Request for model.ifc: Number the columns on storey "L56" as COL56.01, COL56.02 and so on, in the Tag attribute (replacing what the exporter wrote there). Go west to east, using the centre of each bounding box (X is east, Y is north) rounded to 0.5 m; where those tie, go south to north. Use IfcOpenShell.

First a look at what the model holds.

```python
import ifcopenshell
import ifcopenshell.util.element
import ifcopenshell.util.placement

model = ifcopenshell.open("model.ifc")
print(model.schema)
storey = next(s for s in model.by_type("IfcBuildingStorey") if s.Name == "L56")
columns = [e for e in ifcopenshell.util.element.get_decomposition(storey) if e.is_a("IfcColumn")]
for e in sorted(columns, key=lambda e: e.id()):
    origin = ifcopenshell.util.placement.get_local_placement(e.ObjectPlacement)[:3, 3]
    print(e.id(), e.Tag, e.Name, origin.round(2) + 0.0, sep=" | ")
```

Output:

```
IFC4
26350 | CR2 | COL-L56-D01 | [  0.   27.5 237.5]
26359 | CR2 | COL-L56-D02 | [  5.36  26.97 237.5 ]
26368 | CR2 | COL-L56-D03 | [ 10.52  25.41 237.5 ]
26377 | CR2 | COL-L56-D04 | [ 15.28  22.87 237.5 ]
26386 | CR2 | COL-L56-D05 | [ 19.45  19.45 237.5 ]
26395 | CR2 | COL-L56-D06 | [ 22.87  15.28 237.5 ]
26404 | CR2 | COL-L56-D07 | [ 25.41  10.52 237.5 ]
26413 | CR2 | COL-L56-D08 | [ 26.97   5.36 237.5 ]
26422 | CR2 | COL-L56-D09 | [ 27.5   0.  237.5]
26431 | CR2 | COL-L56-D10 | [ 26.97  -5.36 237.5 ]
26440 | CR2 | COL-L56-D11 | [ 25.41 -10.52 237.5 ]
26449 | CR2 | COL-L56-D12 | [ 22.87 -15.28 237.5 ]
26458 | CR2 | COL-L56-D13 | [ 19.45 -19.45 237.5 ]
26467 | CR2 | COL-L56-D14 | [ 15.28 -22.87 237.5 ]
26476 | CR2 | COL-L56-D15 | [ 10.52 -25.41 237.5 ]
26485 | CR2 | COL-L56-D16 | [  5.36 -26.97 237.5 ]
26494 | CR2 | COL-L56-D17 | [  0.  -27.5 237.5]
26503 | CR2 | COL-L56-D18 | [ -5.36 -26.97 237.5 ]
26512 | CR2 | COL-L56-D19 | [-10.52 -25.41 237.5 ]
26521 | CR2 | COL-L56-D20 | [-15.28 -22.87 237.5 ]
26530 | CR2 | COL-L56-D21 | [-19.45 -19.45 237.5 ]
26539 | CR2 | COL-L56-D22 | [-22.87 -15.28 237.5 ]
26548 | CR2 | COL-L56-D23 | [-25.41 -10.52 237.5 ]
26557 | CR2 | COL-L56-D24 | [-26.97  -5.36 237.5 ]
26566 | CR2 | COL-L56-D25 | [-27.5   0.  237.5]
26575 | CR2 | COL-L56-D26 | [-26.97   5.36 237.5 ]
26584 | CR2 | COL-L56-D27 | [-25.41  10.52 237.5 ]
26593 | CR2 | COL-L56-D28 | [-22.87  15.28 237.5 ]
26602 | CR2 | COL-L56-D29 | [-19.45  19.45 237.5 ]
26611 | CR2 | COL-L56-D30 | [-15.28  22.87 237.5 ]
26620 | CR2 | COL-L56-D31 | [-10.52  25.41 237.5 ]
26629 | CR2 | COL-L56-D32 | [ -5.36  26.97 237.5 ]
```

```python
import ifcopenshell
import ifcopenshell.geom
import ifcopenshell.util.element
import ifcopenshell.util.shape

model = ifcopenshell.open("model.ifc")
settings = ifcopenshell.geom.settings()
settings.set("use-world-coords", True)


def centre(element):
    shape = ifcopenshell.geom.create_shape(settings, element)
    return ifcopenshell.util.shape.get_bbox_centroid(shape.geometry)


storey = next(s for s in model.by_type("IfcBuildingStorey") if s.Name == "L56")
columns = [e for e in ifcopenshell.util.element.get_decomposition(storey) if e.is_a("IfcColumn")]

# Insertion points can sit at a corner or the storey origin, so sort by the geometry (in metres).
centres = {e: centre(e) for e in columns}
columns.sort(key=lambda e: (round(centres[e][0] / 0.5), centres[e][1]))

for i, e in enumerate(columns, start=1):
    number = f"COL56.{i:02d}"
    e.Tag = number
    print(e.id(), number)

model.write("model_updated.ifc")
```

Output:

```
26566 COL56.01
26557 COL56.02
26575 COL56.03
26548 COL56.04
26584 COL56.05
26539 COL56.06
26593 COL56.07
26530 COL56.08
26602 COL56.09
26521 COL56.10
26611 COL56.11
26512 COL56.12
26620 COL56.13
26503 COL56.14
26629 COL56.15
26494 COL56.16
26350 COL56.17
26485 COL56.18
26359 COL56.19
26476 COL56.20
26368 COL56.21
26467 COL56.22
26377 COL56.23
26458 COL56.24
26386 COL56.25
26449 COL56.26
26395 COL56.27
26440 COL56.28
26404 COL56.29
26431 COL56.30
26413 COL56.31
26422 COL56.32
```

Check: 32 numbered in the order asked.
